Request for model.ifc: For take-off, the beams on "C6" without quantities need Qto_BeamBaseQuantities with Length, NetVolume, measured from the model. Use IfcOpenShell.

First a look at what the model holds.

```python
import ifcopenshell
import ifcopenshell.util.element
import ifcopenshell.util.unit

model = ifcopenshell.open("model.ifc")
print(model.schema)
for unit_type in ("LENGTHUNIT", "AREAUNIT", "VOLUMEUNIT"):
    print(unit_type, ifcopenshell.util.unit.calculate_unit_scale(model, unit_type))
storey = next(s for s in model.by_type("IfcBuildingStorey") if s.Name == "C6")
beams = [e for e in ifcopenshell.util.element.get_decomposition(storey) if e.is_a("IfcBeam")]
for e in sorted(beams, key=lambda e: e.id()):
    print(e.id(), e.is_a(), e.Name, list(ifcopenshell.util.element.get_psets(e, qtos_only=True)), sep=" | ")
```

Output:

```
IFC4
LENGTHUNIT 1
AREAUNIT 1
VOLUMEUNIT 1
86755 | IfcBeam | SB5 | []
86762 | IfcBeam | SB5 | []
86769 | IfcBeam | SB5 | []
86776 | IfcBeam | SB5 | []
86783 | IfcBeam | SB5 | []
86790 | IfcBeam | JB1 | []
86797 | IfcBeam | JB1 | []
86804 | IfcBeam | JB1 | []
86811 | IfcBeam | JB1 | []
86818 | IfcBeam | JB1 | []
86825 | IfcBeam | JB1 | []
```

```python
import ifcopenshell
import ifcopenshell.api.pset
import ifcopenshell.geom
import ifcopenshell.util.element
import ifcopenshell.util.shape
import ifcopenshell.util.unit

model = ifcopenshell.open("model.ifc")
unit_scale = ifcopenshell.util.unit.calculate_unit_scale(model)
volume_scale = ifcopenshell.util.unit.calculate_unit_scale(model, "VOLUMEUNIT")
settings = ifcopenshell.geom.settings()

storey = next(s for s in model.by_type("IfcBuildingStorey") if s.Name == "C6")
beams = [e for e in ifcopenshell.util.element.get_decomposition(storey) if e.is_a("IfcBeam")]

for e in sorted(beams, key=lambda e: e.id()):
    if ifcopenshell.util.element.get_psets(e, qtos_only=True, should_inherit=False):
        continue
    # Geometry comes back in metres, in the element's own axes.
    shape = ifcopenshell.geom.create_shape(settings, e)
    values = {
        "Length": ifcopenshell.util.shape.get_max_xyz(shape.geometry) / unit_scale,
        "NetVolume": ifcopenshell.util.shape.get_volume(shape.geometry) / volume_scale,
    }
    qto = ifcopenshell.api.pset.add_qto(model, product=e, name="Qto_BeamBaseQuantities")
    ifcopenshell.api.pset.edit_qto(model, qto=qto, properties=values)
    print(e.id(), {k: round(v, 3) for k, v in values.items()})

model.write("model_v2.ifc")
```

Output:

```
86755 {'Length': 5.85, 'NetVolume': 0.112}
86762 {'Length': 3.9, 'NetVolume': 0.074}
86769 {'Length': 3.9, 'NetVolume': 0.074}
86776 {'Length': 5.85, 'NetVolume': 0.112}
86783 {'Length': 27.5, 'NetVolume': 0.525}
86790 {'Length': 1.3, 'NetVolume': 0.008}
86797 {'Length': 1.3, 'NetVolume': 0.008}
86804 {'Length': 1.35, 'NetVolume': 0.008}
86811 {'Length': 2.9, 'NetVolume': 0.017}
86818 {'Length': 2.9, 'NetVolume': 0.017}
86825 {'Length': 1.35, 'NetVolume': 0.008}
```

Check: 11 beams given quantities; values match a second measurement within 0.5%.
